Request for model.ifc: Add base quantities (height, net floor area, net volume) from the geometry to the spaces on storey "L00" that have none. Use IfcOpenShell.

First a look at what the model holds.

```python
import ifcopenshell
import ifcopenshell.util.element
import ifcopenshell.util.unit

model = ifcopenshell.open("model.ifc")
print(model.schema)
for unit_type in ("LENGTHUNIT", "AREAUNIT", "VOLUMEUNIT"):
    print(unit_type, ifcopenshell.util.unit.calculate_unit_scale(model, unit_type))
storey = next(s for s in model.by_type("IfcBuildingStorey") if s.Name == "L00")
spaces = [e for e in ifcopenshell.util.element.get_decomposition(storey) if e.is_a("IfcSpace")]
for e in sorted(spaces, key=lambda e: e.id()):
    print(e.id(), e.is_a(), e.Name, list(ifcopenshell.util.element.get_psets(e, qtos_only=True)), sep=" | ")
```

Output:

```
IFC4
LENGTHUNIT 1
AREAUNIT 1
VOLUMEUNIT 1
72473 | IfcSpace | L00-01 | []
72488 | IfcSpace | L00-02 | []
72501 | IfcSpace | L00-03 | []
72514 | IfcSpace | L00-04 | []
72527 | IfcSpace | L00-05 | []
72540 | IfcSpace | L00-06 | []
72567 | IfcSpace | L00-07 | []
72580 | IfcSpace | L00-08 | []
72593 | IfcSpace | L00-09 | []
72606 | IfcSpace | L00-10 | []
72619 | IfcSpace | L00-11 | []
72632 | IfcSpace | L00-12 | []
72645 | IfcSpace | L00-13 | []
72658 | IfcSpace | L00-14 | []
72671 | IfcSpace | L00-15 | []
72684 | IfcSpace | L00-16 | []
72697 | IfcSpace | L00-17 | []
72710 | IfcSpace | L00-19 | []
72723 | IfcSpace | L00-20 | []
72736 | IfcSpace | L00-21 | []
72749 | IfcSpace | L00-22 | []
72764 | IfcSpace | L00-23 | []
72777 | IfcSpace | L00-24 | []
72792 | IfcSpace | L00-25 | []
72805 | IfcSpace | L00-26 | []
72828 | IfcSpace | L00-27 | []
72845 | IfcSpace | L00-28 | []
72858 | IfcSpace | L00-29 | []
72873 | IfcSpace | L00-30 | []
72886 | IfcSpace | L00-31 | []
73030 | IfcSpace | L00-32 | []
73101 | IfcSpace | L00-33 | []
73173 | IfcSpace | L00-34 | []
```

```python
import ifcopenshell
import ifcopenshell.api.pset
import ifcopenshell.geom
import ifcopenshell.util.element
import ifcopenshell.util.shape
import ifcopenshell.util.unit

model = ifcopenshell.open("model.ifc")
unit_scale = ifcopenshell.util.unit.calculate_unit_scale(model)
area_scale = ifcopenshell.util.unit.calculate_unit_scale(model, "AREAUNIT")
volume_scale = ifcopenshell.util.unit.calculate_unit_scale(model, "VOLUMEUNIT")
settings = ifcopenshell.geom.settings()

storey = next(s for s in model.by_type("IfcBuildingStorey") if s.Name == "L00")
spaces = [e for e in ifcopenshell.util.element.get_decomposition(storey) if e.is_a("IfcSpace")]

for e in sorted(spaces, key=lambda e: e.id()):
    if ifcopenshell.util.element.get_psets(e, qtos_only=True, should_inherit=False):
        continue
    # Geometry comes back in metres, in the element's own axes.
    shape = ifcopenshell.geom.create_shape(settings, e)
    values = {
        "Height": ifcopenshell.util.shape.get_z(shape.geometry) / unit_scale,
        "NetFloorArea": ifcopenshell.util.shape.get_footprint_area(shape.geometry) / area_scale,
        "NetVolume": ifcopenshell.util.shape.get_volume(shape.geometry) / volume_scale,
    }
    qto = ifcopenshell.api.pset.add_qto(model, product=e, name="Qto_SpaceBaseQuantities")
    ifcopenshell.api.pset.edit_qto(model, qto=qto, properties=values)
    print(e.id(), {k: round(v, 3) for k, v in values.items()})

model.write("model_updated.ifc")
```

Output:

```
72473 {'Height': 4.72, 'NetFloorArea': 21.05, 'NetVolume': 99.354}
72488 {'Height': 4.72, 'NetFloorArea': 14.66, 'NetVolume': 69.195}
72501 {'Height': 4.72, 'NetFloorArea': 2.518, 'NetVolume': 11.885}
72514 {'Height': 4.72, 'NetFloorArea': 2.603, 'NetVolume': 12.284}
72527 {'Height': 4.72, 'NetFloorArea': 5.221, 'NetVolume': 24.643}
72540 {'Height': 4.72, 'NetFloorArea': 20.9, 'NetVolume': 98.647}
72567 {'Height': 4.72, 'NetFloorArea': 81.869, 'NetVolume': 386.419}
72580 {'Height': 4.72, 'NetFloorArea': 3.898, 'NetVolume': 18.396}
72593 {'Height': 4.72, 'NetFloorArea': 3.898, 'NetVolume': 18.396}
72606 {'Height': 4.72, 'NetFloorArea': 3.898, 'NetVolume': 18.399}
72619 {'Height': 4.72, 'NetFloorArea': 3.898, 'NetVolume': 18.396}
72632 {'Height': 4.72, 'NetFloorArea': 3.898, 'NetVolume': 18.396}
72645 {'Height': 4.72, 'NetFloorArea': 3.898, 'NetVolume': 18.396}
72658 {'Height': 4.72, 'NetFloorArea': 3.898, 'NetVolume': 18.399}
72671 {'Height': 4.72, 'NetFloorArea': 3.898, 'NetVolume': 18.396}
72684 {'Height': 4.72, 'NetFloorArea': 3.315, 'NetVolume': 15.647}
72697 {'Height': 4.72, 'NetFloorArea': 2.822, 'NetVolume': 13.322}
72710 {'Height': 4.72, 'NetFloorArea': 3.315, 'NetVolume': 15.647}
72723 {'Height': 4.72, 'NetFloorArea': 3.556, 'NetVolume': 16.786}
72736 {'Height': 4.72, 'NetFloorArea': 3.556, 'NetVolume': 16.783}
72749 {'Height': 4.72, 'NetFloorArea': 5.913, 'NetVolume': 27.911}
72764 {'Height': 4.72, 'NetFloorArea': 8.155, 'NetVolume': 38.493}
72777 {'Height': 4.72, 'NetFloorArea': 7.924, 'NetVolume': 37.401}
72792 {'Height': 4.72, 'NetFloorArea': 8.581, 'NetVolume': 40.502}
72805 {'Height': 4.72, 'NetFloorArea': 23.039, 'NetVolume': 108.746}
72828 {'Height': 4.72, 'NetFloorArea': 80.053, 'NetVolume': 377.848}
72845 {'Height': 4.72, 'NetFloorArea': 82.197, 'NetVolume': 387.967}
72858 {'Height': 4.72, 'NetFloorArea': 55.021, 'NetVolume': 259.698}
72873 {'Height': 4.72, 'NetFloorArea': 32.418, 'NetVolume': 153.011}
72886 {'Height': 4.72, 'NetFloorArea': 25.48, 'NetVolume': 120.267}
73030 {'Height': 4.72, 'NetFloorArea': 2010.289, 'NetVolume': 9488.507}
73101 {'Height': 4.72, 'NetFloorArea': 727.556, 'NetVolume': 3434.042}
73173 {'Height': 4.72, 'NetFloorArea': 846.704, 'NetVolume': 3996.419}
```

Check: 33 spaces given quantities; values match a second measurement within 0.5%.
